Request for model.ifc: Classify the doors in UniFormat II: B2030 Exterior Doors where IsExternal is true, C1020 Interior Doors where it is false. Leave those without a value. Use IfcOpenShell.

First a look at what the model holds.

```python
import ifcopenshell
import ifcopenshell.util.element

model = ifcopenshell.open("model.ifc")
print(model.schema)
print("classifications:", [c.Name for c in model.by_type("IfcClassification")])
values = [ifcopenshell.util.element.get_pset(e, "Pset_DoorCommon", "IsExternal") for e in model.by_type("IfcDoor")]
for value in (True, False, None):
    print("IsExternal", value, values.count(value))
```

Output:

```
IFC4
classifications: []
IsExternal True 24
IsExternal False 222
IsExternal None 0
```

```python
import ifcopenshell
import ifcopenshell.api.classification
import ifcopenshell.util.element

model = ifcopenshell.open("model.ifc")

system = ifcopenshell.api.classification.add_classification(model, classification="UniFormat II")

doors = model.by_type("IfcDoor")
external = {e: ifcopenshell.util.element.get_pset(e, "Pset_DoorCommon", "IsExternal") for e in doors}
for flag, code, name in ((True, "B2030", "Exterior Doors"), (False, "C1020", "Interior Doors")):
    products = [e for e in doors if external[e] is flag]
    ifcopenshell.api.classification.add_reference(
        model, products=products, classification=system, identification=code, name=name
    )
    print(code, len(products))

model.write("model_rev.ifc")
```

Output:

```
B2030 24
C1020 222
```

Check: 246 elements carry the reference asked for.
